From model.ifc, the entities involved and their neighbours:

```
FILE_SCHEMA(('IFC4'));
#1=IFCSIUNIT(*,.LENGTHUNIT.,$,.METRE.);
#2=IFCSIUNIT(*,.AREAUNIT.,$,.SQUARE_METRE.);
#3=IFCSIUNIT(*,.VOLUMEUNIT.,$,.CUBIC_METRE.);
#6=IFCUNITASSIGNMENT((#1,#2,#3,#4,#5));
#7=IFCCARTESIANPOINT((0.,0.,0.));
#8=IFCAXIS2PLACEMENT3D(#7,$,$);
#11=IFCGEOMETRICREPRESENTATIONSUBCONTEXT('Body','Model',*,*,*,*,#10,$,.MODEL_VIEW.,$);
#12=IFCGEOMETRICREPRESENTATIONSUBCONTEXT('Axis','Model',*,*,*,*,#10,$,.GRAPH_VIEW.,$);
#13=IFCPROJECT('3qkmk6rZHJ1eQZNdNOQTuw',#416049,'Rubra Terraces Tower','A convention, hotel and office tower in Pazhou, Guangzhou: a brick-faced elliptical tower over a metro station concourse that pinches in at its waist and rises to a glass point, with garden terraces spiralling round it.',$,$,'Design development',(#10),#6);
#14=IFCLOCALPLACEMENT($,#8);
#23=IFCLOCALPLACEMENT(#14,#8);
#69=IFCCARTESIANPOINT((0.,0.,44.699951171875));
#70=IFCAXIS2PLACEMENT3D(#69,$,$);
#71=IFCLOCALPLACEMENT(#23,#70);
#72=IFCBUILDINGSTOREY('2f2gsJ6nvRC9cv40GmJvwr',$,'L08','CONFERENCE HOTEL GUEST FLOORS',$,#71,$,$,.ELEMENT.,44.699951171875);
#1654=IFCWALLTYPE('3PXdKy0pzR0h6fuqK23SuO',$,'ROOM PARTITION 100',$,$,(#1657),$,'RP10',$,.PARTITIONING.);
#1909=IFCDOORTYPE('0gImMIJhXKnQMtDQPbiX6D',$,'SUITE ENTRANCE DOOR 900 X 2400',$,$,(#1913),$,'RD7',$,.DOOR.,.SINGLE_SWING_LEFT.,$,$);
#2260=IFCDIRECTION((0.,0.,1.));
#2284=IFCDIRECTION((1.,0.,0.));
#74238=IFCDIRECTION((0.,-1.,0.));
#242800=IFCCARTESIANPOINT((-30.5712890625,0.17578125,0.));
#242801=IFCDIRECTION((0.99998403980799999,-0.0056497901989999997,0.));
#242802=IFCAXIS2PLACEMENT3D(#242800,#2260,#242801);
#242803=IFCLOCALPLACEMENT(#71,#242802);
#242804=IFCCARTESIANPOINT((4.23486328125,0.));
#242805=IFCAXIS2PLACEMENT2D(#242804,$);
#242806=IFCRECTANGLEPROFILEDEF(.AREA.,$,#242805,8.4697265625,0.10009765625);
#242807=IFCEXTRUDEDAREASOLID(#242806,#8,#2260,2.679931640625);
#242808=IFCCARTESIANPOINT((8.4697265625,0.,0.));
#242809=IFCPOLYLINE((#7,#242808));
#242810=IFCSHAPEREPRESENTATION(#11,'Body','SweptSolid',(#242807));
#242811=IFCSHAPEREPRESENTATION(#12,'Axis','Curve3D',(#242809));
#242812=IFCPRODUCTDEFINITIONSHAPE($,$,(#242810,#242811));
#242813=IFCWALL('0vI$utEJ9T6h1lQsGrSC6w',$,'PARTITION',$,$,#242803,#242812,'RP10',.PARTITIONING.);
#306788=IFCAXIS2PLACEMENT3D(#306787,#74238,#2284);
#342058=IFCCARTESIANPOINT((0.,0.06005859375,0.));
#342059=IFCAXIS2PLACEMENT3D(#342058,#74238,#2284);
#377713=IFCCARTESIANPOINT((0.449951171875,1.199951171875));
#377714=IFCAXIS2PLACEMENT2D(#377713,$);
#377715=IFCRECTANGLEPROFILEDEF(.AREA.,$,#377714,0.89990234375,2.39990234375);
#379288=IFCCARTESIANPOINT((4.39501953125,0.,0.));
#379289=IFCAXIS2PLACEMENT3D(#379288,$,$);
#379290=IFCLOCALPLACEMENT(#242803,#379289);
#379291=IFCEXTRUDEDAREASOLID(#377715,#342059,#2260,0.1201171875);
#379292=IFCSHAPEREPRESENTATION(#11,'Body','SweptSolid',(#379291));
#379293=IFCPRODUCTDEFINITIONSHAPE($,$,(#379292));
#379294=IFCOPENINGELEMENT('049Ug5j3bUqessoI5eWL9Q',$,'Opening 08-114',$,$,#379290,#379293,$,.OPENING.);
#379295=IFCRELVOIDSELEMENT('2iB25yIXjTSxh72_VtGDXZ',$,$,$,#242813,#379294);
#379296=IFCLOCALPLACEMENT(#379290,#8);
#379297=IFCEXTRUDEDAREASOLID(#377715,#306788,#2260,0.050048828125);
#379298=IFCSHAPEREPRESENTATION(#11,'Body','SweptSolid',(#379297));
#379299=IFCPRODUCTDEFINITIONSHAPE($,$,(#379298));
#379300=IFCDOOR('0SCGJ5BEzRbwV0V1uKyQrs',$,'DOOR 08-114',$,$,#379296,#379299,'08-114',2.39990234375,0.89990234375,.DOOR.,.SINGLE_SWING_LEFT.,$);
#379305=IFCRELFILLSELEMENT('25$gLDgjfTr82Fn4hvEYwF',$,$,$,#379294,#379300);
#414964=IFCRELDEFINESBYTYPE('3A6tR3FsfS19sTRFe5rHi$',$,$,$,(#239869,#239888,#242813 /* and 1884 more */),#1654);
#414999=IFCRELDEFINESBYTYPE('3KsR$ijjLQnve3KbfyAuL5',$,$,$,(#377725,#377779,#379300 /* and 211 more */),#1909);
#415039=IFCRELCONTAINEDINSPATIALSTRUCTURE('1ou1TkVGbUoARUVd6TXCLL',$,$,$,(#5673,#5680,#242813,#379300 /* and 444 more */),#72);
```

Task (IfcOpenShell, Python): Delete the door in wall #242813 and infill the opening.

```python
import ifcopenshell
import ifcopenshell.api.feature
import ifcopenshell.api.root
import ifcopenshell.geom
import ifcopenshell.util.shape

model = ifcopenshell.open("model.ifc")
settings = ifcopenshell.geom.settings()


def volume(element):
    """Net volume in cubic metres, openings subtracted."""
    shape = ifcopenshell.geom.create_shape(settings, element)
    return ifcopenshell.util.shape.get_volume(shape.geometry)


door = model.by_guid("0SCGJ5BEzRbwV0V1uKyQrs")
opening = door.FillsVoids[0].RelatingOpeningElement
wall = opening.VoidsElements[0].RelatingBuildingElement
before = volume(wall)

ifcopenshell.api.root.remove_product(model, product=door)
ifcopenshell.api.feature.remove_feature(model, feature=opening)

after = volume(wall)

print(f"wall volume {before:.3f} -> {after:.3f} m3")

model.write("model_rev.ifc")
```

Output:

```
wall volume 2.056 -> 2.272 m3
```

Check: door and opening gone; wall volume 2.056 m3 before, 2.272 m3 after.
